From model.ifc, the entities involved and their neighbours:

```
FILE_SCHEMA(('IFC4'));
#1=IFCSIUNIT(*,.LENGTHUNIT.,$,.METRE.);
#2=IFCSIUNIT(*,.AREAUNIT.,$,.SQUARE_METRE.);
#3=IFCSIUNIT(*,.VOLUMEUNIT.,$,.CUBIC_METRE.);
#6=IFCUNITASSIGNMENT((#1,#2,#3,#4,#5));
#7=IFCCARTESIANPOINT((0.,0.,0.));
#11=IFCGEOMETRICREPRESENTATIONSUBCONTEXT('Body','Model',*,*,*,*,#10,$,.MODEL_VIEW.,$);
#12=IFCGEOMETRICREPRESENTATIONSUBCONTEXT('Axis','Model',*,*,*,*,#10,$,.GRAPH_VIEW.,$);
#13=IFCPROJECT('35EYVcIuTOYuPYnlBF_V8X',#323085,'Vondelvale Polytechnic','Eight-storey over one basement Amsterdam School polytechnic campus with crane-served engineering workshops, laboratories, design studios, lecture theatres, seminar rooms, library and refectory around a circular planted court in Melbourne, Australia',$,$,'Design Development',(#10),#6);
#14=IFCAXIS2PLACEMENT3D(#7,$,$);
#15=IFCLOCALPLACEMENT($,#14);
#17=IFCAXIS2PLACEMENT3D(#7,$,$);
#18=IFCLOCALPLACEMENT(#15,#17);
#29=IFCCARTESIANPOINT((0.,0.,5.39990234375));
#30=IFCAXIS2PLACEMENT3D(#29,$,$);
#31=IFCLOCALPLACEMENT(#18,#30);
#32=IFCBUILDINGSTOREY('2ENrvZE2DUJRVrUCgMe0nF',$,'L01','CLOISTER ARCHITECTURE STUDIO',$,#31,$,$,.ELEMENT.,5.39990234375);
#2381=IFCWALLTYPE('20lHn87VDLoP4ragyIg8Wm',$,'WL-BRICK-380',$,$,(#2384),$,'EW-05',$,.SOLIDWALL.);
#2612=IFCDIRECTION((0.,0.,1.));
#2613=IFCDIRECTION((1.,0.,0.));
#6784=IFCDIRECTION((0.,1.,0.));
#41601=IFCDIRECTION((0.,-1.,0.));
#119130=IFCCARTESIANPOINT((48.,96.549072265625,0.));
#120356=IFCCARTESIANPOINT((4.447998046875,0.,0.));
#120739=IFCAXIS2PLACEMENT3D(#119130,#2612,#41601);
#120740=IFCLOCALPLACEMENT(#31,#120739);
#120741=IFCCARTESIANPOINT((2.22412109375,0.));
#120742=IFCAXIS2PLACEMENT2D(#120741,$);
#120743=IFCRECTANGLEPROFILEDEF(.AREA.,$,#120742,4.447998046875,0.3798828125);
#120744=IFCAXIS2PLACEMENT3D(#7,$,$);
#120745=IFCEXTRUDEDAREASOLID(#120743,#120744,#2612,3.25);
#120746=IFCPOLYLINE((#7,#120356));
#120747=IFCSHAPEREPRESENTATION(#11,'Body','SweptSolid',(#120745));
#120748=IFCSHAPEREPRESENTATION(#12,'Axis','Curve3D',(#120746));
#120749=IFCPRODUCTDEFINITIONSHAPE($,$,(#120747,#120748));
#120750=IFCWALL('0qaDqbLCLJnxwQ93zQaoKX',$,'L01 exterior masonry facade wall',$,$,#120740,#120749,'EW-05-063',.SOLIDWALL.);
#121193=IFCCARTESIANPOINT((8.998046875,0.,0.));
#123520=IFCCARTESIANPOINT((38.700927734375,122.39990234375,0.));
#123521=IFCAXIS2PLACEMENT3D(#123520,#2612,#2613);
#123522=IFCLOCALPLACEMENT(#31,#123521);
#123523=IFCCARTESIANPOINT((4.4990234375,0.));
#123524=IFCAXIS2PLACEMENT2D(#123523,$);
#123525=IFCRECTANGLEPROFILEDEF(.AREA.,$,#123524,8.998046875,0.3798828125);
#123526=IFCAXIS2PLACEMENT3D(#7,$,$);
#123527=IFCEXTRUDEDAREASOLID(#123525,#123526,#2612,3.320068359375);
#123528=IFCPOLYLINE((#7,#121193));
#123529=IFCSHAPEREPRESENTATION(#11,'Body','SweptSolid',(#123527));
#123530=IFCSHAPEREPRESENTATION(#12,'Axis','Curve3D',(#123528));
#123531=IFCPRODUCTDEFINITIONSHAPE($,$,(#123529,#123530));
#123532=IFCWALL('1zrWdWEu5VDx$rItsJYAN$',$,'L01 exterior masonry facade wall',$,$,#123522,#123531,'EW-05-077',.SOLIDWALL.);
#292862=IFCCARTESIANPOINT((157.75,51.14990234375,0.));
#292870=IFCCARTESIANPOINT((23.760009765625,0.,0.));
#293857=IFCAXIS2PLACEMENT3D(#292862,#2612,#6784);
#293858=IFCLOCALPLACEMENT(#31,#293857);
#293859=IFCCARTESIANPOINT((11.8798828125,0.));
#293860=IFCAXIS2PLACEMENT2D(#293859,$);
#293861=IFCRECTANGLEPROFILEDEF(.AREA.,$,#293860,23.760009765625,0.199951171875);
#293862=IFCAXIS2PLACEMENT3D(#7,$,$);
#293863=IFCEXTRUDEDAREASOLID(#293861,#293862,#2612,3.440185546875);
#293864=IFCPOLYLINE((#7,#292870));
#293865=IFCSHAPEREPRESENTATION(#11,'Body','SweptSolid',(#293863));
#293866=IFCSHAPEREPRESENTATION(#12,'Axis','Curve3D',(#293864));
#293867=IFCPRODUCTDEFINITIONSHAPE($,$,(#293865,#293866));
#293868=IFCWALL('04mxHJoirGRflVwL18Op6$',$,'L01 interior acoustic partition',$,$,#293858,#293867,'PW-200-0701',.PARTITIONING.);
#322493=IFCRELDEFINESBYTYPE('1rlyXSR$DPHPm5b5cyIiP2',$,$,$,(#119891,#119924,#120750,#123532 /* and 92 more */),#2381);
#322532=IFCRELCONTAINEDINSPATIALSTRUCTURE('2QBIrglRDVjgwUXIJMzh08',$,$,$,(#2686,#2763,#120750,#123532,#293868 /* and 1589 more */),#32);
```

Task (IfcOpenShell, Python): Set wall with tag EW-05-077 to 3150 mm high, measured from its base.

```python
import ifcopenshell
import ifcopenshell.geom
import ifcopenshell.util.representation
import ifcopenshell.util.shape

model = ifcopenshell.open("model.ifc")
settings = ifcopenshell.geom.settings()


def volume(element):
    """Net volume in cubic metres, openings subtracted."""
    shape = ifcopenshell.geom.create_shape(settings, element)
    return ifcopenshell.util.shape.get_volume(shape.geometry)


wall = model.by_guid("1zrWdWEu5VDx$rItsJYAN$")
before = volume(wall)

body = ifcopenshell.util.representation.get_representation(wall, "Model", "Body")
solid = body.Items[0]
old_height = solid.Depth
solid.Depth = 3.15
after = volume(wall)

print(f"height {old_height:g} -> {solid.Depth:g}, volume {before:.3f} -> {after:.3f} m3")

model.write("model_rev.ifc")
```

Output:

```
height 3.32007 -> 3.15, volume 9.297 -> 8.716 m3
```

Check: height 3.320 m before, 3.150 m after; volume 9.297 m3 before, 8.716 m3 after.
